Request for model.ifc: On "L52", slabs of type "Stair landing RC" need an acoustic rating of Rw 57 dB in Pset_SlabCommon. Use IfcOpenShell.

First a look at what the model holds.

```python
import ifcopenshell
import ifcopenshell.util.element

model = ifcopenshell.open("model.ifc")
print(model.schema)
storey = next(s for s in model.by_type("IfcBuildingStorey") if s.Name == "L52")
slabs = [e for e in ifcopenshell.util.element.get_decomposition(storey) if e.is_a("IfcSlab")]
seen = {}
for e in slabs:
    element_type = ifcopenshell.util.element.get_type(e)
    key = (element_type.Name if element_type != e and element_type else None, ifcopenshell.util.element.get_pset(e, "Pset_SlabCommon", "AcousticRating"))
    seen[key] = seen.get(key, 0) + 1
for (name, value), count in sorted(seen.items(), key=str):
    print(count, "x", name, "|", value)
```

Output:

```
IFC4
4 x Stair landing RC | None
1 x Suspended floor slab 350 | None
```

```python
import ifcopenshell
import ifcopenshell.api.pset
import ifcopenshell.util.element

model = ifcopenshell.open("model.ifc")

storey = next(s for s in model.by_type("IfcBuildingStorey") if s.Name == "L52")
slabs = [e for e in ifcopenshell.util.element.get_decomposition(storey) if e.is_a("IfcSlab")]

count = 0
for e in slabs:
    element_type = ifcopenshell.util.element.get_type(e)
    if element_type in (None, e) or element_type.Name != "Stair landing RC":
        continue
    # add_pset returns the element's existing set when there is one.
    pset = ifcopenshell.api.pset.add_pset(model, product=e, name="Pset_SlabCommon")
    ifcopenshell.api.pset.edit_pset(model, pset=pset, properties={"AcousticRating": "Rw 57 dB"})
    count += 1

print(count, "slabs updated")

model.write("model_rev.ifc")
```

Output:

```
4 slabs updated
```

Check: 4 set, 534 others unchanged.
